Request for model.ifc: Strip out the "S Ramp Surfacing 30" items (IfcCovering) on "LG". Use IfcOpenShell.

First a look at what the model holds.

```python
import ifcopenshell
import ifcopenshell.util.element

model = ifcopenshell.open("model.ifc")
print(model.schema)
storey = next(s for s in model.by_type("IfcBuildingStorey") if s.Name == "LG")
coverings = [e for e in ifcopenshell.util.element.get_decomposition(storey) if e.is_a("IfcCovering")]
seen = {}
for e in coverings:
    element_type = ifcopenshell.util.element.get_type(e)
    name = element_type.Name if element_type not in (None, e) else None
    seen[name] = seen.get(name, 0) + 1
for name, count in sorted(seen.items(), key=str):
    print(count, "x", name)
```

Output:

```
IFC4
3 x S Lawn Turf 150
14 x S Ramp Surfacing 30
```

```python
import ifcopenshell
import ifcopenshell.api.root
import ifcopenshell.util.element

model = ifcopenshell.open("model.ifc")

storey = next(s for s in model.by_type("IfcBuildingStorey") if s.Name == "LG")
coverings = [e for e in ifcopenshell.util.element.get_decomposition(storey) if e.is_a("IfcCovering")]
targets = [e for e in coverings if (t := ifcopenshell.util.element.get_type(e)) not in (None, e) and t.Name == "S Ramp Surfacing 30"]

for e in targets:
    ifcopenshell.api.root.remove_product(model, product=e)
print(len(targets), "removed")

model.write("model_rev.ifc")
```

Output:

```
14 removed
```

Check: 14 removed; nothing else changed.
